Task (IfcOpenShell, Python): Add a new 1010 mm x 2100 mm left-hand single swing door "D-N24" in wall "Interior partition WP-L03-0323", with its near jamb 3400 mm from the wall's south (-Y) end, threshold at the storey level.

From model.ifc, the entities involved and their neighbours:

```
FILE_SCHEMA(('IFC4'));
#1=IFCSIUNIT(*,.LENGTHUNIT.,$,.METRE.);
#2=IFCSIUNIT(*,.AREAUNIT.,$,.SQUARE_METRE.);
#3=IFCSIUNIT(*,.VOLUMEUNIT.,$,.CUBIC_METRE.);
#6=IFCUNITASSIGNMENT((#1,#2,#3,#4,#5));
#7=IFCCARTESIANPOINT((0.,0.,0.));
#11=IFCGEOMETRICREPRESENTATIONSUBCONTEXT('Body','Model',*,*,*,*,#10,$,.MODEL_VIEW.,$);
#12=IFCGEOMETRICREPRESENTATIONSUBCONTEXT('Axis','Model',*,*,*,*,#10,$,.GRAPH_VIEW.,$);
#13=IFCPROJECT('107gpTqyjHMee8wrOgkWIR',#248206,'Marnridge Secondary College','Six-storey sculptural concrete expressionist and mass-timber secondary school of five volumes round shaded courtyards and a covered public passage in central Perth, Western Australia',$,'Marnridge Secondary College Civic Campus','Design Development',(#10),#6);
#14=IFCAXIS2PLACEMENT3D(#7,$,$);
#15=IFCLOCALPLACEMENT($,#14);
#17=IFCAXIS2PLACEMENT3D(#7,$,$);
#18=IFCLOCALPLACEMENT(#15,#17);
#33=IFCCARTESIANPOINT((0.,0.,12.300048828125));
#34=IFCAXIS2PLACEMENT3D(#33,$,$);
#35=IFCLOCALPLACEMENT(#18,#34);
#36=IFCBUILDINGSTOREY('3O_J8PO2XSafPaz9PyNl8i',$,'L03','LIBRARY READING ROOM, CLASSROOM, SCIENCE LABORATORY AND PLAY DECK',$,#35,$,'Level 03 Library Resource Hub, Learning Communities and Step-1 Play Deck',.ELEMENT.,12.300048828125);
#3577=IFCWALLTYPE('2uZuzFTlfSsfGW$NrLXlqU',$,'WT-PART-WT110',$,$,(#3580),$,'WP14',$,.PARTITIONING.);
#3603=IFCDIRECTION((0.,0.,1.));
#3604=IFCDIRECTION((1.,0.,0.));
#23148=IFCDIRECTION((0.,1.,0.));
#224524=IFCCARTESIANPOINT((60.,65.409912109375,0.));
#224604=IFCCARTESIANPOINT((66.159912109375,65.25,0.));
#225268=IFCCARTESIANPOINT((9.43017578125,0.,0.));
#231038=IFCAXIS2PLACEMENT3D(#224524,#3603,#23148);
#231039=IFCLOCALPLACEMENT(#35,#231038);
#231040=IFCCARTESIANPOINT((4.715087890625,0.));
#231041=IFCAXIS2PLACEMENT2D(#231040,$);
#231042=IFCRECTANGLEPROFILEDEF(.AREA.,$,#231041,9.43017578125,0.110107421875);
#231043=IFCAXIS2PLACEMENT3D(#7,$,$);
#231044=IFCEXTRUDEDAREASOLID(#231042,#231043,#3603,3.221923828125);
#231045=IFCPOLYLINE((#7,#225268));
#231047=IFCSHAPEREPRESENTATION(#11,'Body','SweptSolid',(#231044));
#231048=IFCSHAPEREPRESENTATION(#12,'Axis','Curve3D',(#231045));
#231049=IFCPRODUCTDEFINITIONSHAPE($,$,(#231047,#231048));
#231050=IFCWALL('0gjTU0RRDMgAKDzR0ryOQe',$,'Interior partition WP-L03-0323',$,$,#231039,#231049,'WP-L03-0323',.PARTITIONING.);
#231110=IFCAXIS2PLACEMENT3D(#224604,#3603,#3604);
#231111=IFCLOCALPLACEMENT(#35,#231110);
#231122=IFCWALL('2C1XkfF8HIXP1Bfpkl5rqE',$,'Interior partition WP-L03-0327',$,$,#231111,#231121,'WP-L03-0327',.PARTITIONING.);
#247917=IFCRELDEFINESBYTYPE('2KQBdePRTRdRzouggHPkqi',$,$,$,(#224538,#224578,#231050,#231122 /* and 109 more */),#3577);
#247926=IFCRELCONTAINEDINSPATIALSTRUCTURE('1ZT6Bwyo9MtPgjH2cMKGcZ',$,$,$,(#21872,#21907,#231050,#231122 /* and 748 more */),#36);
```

```python
import numpy as np
import ifcopenshell
import ifcopenshell.api.feature
import ifcopenshell.api.geometry
import ifcopenshell.api.root
import ifcopenshell.api.spatial
import ifcopenshell.geom
import ifcopenshell.util.element
import ifcopenshell.util.placement
import ifcopenshell.util.representation
import ifcopenshell.util.shape
import ifcopenshell.util.unit

model = ifcopenshell.open("model.ifc")
unit_scale = ifcopenshell.util.unit.calculate_unit_scale(model)
settings = ifcopenshell.geom.settings()


def volume(element):
    """Net volume in cubic metres, openings subtracted."""
    shape = ifcopenshell.geom.create_shape(settings, element)
    return ifcopenshell.util.shape.get_volume(shape.geometry)


wall = model.by_guid("0gjTU0RRDMgAKDzR0ryOQe")
storey = ifcopenshell.util.element.get_container(wall, ifc_class="IfcBuildingStorey")
context = ifcopenshell.util.representation.get_context(model, "Model", "Body", "MODEL_VIEW")
before = volume(wall)

width, height, from_end, sill = 1.01, 2.1, 3.4, 0.0  # metres

# The wall runs along its own X axis, and the end named is its -X end.
wall_shape = ifcopenshell.geom.create_shape(settings, wall)
x, y, z = ifcopenshell.util.shape.get_vertices(wall_shape.geometry).T
start = x.min() + from_end
face, thickness = float(y.min()), float(y.max() - y.min())
wall_matrix = ifcopenshell.util.placement.get_local_placement(wall.ObjectPlacement)
level = ifcopenshell.util.placement.get_local_placement(storey.ObjectPlacement)[2, 3]


def in_wall(x, y):
    """Placement at x, y metres in the wall's axes, at sill height."""
    matrix = wall_matrix.copy()
    matrix[:, 3] = wall_matrix @ np.array([x / unit_scale, y / unit_scale, 0.0, 1.0])
    matrix[2, 3] = level + sill / unit_scale
    return matrix


# Opening: a box that overshoots both wall faces by 50 mm.
opening = ifcopenshell.api.root.create_entity(model, ifc_class="IfcOpeningElement", predefined_type="OPENING")
box = ifcopenshell.api.geometry.add_wall_representation(
    model, context=context, length=width, height=height, thickness=thickness + 0.1
)
ifcopenshell.api.geometry.assign_representation(model, product=opening, representation=box)
ifcopenshell.api.geometry.edit_object_placement(model, product=opening, matrix=in_wall(start, face - 0.05), is_si=False)
ifcopenshell.api.feature.add_feature(model, feature=opening, element=wall)

door = ifcopenshell.api.root.create_entity(model, ifc_class="IfcDoor", name="D-N24", predefined_type="DOOR")
door.OverallWidth, door.OverallHeight = width / unit_scale, height / unit_scale
door.OperationType = "SINGLE_SWING_LEFT"
body = ifcopenshell.api.geometry.add_door_representation(
    model,
    context=context,
    overall_width=door.OverallWidth,
    overall_height=door.OverallHeight,
    operation_type="SINGLE_SWING_LEFT",
    lining_properties={"LiningDepth": thickness / unit_scale, "ThresholdDepth": thickness / unit_scale},
)
ifcopenshell.api.geometry.assign_representation(model, product=door, representation=body)
ifcopenshell.api.spatial.assign_container(model, products=[door], relating_structure=storey)
ifcopenshell.api.feature.add_filling(model, opening=opening, element=door)

# The lining spans the wall, so the door starts at the wall face.
ifcopenshell.api.geometry.edit_object_placement(model, product=door, matrix=in_wall(start, face), is_si=False)

after = volume(wall)

print(f"wall volume {before:.3f} -> {after:.3f} m3")

model.write("model_edited.ifc")
```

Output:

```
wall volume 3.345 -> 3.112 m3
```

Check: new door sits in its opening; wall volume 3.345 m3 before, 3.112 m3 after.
